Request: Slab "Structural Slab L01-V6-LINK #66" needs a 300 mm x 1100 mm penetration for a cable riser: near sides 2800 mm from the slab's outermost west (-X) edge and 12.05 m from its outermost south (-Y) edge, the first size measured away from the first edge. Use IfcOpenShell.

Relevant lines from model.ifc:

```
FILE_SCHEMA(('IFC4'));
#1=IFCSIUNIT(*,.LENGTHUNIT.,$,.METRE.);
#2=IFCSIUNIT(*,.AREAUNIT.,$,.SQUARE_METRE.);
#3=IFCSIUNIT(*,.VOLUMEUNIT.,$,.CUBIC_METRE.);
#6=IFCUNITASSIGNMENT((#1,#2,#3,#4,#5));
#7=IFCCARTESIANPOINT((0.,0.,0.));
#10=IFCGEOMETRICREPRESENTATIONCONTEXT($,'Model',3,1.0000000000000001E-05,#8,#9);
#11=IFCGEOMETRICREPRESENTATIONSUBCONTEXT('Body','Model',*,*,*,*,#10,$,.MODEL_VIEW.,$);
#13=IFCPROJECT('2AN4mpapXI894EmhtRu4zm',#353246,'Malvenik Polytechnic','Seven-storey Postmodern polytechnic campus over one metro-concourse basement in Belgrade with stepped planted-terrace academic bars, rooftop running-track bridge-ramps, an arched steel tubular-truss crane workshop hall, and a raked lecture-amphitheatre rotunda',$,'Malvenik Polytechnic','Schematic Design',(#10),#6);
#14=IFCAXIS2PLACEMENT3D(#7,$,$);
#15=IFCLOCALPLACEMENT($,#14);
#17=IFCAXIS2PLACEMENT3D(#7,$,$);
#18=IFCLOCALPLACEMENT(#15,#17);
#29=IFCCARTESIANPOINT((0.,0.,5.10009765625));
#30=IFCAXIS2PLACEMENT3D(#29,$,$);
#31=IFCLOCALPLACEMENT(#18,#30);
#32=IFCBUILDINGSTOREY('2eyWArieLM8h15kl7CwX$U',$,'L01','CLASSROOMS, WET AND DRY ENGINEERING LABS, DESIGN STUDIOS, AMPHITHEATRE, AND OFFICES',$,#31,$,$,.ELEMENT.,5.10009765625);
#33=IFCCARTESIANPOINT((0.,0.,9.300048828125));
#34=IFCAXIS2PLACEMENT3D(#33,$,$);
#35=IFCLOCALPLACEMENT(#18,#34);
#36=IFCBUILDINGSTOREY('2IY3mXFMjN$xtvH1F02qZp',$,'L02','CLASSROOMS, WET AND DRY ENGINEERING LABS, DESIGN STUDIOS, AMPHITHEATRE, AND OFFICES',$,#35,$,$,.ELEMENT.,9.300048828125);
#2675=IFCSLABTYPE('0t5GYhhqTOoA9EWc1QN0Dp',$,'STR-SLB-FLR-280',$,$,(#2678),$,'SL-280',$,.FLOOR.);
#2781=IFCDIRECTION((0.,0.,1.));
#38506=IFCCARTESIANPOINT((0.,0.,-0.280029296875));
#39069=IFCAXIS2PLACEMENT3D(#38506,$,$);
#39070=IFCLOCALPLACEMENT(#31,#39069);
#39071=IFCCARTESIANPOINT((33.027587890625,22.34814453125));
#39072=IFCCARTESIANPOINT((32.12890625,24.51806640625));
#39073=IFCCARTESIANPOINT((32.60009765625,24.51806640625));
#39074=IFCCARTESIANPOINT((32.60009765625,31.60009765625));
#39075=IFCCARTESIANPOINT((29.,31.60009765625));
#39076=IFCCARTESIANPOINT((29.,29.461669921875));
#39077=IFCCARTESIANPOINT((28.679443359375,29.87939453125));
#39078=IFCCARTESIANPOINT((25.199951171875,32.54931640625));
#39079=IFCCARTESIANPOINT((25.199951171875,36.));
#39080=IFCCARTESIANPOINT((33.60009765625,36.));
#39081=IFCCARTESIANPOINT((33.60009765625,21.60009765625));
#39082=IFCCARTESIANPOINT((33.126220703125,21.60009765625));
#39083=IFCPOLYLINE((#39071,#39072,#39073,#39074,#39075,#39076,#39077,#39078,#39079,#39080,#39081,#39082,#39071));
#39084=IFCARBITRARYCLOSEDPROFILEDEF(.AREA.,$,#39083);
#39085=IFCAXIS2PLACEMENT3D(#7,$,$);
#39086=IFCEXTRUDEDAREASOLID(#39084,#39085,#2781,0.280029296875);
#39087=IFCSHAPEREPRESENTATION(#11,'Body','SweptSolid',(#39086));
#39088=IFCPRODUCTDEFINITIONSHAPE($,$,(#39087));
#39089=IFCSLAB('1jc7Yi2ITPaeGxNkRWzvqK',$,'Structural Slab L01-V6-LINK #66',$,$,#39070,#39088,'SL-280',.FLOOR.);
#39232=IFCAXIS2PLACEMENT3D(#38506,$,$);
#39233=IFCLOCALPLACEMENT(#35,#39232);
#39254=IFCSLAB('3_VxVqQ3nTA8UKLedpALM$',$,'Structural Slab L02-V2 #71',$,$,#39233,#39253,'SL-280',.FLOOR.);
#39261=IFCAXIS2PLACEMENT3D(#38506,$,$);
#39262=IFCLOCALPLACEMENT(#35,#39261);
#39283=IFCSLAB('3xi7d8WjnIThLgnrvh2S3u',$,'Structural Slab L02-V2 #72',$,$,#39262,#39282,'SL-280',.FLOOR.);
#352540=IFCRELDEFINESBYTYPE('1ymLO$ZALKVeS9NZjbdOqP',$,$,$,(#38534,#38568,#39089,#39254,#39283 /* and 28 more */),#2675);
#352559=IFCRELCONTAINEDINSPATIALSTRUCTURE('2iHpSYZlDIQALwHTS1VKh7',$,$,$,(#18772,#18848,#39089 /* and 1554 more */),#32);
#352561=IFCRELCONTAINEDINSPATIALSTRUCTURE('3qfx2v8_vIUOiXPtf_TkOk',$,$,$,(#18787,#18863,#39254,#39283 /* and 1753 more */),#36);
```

```python
import numpy as np
import ifcopenshell
import ifcopenshell.api.feature
import ifcopenshell.api.geometry
import ifcopenshell.api.root
import ifcopenshell.geom
import ifcopenshell.util.placement
import ifcopenshell.util.representation
import ifcopenshell.util.shape
import ifcopenshell.util.unit

model = ifcopenshell.open("model.ifc")
unit_scale = ifcopenshell.util.unit.calculate_unit_scale(model)
settings = ifcopenshell.geom.settings()


def volume(element):
    """Net volume in cubic metres, openings subtracted."""
    shape = ifcopenshell.geom.create_shape(settings, element)
    return ifcopenshell.util.shape.get_volume(shape.geometry)


slab = model.by_guid("1jc7Yi2ITPaeGxNkRWzvqK")
before = volume(slab)

# Extent in the slab's own axes, in metres. The edges named are its -X and -Y sides.
slab_shape = ifcopenshell.geom.create_shape(settings, slab)
vertices = ifcopenshell.util.shape.get_vertices(slab_shape.geometry)
x_min, y_min, bottom = vertices.min(axis=0)
top = vertices[:, 2].max()

opening = ifcopenshell.api.root.create_entity(model, ifc_class="IfcOpeningElement", name="Cable riser opening", predefined_type="OPENING")
context = ifcopenshell.util.representation.get_context(model, "Model", "Body", "MODEL_VIEW")
width, depth = 0.3, 1.1
outline = [(0.0, 0.0), (width, 0.0), (width, depth), (0.0, depth), (0.0, 0.0)]
# Overshoot both faces by 50 mm so the cut is clean.
shape = ifcopenshell.api.geometry.add_slab_representation(
    model, context=context, depth=top - bottom + 0.1, polyline=outline
)
ifcopenshell.api.geometry.assign_representation(model, product=opening, representation=shape)

matrix = ifcopenshell.util.placement.get_local_placement(slab.ObjectPlacement)
matrix[:, 3] = matrix @ np.append(np.array([x_min + 2.8, y_min + 12.05, bottom - 0.05]) / unit_scale, 1.0)
ifcopenshell.api.geometry.edit_object_placement(model, product=opening, matrix=matrix, is_si=False)
ifcopenshell.api.feature.add_feature(model, feature=opening, element=slab)

after = volume(slab)

print(f"slab volume {before:.3f} -> {after:.3f} m3")

model.write("model_v2.ifc")
```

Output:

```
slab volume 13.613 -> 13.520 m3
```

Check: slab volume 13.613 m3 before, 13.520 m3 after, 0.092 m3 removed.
